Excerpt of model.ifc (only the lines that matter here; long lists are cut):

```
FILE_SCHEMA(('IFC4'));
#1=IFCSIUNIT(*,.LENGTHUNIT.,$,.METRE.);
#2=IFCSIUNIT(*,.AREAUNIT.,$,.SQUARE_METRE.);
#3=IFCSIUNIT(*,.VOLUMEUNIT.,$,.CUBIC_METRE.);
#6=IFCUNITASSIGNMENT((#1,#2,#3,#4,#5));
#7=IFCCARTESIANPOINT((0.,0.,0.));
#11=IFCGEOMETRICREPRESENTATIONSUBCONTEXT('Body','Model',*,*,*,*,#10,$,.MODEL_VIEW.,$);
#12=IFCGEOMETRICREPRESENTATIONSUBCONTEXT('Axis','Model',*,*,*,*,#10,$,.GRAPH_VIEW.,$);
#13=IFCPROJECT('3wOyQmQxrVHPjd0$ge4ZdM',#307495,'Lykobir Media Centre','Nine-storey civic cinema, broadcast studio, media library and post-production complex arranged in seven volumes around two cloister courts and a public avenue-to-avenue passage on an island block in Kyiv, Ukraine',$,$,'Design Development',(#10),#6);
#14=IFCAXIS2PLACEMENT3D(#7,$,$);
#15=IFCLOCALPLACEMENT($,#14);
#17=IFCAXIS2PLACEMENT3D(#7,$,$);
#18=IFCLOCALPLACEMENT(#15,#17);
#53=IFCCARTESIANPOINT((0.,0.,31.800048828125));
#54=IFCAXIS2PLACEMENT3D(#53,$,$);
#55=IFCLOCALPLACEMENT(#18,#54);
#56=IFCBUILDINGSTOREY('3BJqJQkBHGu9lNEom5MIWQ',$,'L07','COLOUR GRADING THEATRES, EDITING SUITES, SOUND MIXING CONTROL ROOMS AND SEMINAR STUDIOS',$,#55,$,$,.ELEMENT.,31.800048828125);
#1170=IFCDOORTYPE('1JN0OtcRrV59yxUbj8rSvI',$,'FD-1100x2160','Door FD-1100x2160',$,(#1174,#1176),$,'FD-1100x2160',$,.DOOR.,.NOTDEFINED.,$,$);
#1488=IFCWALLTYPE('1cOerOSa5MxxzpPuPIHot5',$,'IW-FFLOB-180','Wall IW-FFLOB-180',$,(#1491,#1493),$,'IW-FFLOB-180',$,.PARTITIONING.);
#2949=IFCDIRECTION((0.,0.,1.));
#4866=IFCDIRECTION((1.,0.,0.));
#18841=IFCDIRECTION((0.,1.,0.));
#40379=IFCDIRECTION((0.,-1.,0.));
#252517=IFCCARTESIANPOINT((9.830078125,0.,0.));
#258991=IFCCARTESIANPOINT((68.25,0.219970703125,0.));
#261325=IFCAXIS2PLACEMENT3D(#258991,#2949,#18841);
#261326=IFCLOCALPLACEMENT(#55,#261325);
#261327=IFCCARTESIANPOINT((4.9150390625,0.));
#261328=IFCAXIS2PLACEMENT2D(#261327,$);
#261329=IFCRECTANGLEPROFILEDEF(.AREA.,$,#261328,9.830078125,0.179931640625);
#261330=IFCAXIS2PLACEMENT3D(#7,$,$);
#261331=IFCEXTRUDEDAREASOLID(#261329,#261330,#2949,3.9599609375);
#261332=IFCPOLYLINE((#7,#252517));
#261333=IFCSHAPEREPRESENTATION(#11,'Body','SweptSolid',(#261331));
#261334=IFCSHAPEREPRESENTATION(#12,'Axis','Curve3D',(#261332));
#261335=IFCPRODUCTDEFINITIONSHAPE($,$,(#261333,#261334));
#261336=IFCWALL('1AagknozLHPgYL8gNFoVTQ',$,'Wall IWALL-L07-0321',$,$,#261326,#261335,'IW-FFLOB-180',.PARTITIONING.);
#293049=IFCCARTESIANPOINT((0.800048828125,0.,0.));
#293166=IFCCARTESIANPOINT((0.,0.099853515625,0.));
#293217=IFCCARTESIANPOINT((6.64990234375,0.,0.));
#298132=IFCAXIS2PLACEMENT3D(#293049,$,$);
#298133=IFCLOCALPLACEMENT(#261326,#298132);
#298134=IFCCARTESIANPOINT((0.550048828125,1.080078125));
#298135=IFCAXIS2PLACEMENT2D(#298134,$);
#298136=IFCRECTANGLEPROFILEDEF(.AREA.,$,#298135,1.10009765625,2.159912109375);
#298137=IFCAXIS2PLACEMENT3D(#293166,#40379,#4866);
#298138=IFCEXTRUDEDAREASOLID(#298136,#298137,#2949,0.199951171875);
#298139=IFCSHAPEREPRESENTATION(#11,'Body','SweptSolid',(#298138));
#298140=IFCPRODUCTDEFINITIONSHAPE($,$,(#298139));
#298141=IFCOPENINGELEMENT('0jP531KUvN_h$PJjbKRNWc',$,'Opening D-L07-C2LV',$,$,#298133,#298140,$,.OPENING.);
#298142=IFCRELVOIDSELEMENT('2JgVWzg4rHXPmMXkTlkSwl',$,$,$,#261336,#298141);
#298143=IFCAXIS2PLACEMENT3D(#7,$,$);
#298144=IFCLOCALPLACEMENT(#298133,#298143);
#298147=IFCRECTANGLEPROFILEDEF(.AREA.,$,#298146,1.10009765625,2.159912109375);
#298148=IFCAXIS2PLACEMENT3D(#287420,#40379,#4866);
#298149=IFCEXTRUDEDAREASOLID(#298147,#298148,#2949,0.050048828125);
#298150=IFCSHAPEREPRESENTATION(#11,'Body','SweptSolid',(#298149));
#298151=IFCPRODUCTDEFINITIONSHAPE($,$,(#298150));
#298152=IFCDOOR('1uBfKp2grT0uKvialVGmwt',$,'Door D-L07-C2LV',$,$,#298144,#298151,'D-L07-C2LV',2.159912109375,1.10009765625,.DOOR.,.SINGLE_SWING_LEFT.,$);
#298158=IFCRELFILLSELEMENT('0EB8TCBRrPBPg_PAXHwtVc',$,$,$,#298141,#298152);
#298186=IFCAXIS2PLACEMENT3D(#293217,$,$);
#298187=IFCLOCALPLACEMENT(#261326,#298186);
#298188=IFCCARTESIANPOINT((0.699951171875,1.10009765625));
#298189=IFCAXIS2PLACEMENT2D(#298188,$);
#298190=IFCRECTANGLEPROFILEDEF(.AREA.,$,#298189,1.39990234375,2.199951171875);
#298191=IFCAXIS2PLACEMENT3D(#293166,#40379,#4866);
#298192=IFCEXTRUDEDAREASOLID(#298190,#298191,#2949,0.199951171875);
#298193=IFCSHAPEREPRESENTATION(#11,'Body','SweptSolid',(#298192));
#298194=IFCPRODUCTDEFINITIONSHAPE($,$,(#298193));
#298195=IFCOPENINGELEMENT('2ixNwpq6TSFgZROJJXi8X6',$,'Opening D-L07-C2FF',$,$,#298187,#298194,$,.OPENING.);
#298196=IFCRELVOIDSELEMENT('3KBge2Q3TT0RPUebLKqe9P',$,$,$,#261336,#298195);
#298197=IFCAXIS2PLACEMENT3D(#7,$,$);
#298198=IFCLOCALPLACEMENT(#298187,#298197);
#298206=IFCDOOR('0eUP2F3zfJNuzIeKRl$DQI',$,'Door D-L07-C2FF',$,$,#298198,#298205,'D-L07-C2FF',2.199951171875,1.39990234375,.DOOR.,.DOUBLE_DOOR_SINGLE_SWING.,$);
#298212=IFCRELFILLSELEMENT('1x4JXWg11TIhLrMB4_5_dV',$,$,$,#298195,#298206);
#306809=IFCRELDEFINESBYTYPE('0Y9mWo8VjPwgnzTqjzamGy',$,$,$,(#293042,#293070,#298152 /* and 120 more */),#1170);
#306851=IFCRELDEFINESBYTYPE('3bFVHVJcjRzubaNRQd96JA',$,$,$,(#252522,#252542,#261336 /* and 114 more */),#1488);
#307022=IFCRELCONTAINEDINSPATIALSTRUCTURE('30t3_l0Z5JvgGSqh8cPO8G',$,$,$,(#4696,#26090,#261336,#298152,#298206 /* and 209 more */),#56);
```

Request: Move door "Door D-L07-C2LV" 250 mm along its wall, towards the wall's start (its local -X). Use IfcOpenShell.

```python
import ifcopenshell
import ifcopenshell.api.geometry
import ifcopenshell.util.placement
import ifcopenshell.util.unit

model = ifcopenshell.open("model.ifc")
unit_scale = ifcopenshell.util.unit.calculate_unit_scale(model)

door = model.by_guid("1uBfKp2grT0uKvialVGmwt")
opening = door.FillsVoids[0].RelatingOpeningElement
wall = opening.VoidsElements[0].RelatingBuildingElement

wall_matrix = ifcopenshell.util.placement.get_local_placement(wall.ObjectPlacement)
shift = wall_matrix[:3, 0] * -0.25 / unit_scale
before = ifcopenshell.util.placement.get_local_placement(door.ObjectPlacement)[:3, 3].copy()

# The door is placed relative to its opening, so it follows when the opening moves.
matrix = ifcopenshell.util.placement.get_local_placement(opening.ObjectPlacement)
matrix[:3, 3] += shift
ifcopenshell.api.geometry.edit_object_placement(
    model, product=opening, matrix=matrix, is_si=False, should_transform_children=True
)

after = ifcopenshell.util.placement.get_local_placement(door.ObjectPlacement)[:3, 3]
print("door moved by", (after - before).round(3) + 0.0)

model.write("model-out.ifc")
```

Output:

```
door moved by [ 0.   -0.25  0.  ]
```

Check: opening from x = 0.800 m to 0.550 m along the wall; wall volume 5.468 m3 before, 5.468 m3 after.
